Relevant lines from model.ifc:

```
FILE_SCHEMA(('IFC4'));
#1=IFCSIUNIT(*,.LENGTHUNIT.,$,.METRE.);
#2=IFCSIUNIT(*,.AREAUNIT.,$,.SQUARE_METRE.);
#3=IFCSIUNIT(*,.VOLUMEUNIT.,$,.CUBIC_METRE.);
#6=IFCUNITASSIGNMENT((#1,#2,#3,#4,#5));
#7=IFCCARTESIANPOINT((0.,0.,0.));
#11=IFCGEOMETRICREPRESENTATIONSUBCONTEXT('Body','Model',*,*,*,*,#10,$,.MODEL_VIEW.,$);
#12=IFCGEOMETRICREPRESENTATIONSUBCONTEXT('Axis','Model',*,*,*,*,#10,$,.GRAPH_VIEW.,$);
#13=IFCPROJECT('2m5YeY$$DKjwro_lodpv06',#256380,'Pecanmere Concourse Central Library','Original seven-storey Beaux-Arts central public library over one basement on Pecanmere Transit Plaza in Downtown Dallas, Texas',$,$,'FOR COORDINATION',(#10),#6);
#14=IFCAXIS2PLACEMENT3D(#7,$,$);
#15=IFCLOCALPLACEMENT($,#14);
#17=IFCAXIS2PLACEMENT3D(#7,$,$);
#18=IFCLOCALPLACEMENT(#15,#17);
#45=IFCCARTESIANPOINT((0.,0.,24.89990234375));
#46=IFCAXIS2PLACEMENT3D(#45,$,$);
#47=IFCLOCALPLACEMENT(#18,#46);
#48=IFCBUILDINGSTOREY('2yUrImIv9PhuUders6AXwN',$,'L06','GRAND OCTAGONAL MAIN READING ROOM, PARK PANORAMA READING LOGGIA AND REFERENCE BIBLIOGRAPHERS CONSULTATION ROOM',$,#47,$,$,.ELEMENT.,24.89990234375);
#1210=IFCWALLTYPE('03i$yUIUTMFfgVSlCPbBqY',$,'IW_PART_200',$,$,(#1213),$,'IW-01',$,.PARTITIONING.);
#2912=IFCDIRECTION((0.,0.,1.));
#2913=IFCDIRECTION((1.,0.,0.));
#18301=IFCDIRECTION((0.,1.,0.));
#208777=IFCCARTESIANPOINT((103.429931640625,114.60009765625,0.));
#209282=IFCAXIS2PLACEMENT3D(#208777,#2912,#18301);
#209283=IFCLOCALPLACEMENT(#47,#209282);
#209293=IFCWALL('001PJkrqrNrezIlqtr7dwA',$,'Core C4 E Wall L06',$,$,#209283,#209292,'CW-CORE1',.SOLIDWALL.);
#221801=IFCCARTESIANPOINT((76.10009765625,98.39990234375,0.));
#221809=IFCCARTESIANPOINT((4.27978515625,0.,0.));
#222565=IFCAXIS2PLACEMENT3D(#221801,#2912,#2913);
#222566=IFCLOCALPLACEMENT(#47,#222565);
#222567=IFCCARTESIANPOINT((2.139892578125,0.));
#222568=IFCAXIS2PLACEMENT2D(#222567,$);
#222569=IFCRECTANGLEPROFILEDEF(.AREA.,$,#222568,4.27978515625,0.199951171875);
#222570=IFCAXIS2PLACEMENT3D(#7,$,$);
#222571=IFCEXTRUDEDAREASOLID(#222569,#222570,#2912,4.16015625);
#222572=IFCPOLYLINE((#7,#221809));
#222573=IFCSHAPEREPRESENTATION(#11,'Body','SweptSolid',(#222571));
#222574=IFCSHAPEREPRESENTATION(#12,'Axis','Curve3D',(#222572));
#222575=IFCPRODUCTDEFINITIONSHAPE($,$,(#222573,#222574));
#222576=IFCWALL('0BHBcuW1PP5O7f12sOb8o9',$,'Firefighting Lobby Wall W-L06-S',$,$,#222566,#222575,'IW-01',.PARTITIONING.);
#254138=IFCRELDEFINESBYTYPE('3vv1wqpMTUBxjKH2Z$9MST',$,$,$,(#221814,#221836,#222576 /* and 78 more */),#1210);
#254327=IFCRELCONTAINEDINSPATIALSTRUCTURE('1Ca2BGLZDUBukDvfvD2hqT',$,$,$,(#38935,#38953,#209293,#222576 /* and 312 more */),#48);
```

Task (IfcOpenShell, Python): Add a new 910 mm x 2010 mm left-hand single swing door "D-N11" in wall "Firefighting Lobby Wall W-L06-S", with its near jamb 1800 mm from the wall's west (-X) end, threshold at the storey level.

```python
import numpy as np
import ifcopenshell
import ifcopenshell.api.feature
import ifcopenshell.api.geometry
import ifcopenshell.api.root
import ifcopenshell.api.spatial
import ifcopenshell.geom
import ifcopenshell.util.element
import ifcopenshell.util.placement
import ifcopenshell.util.representation
import ifcopenshell.util.shape
import ifcopenshell.util.unit

model = ifcopenshell.open("model.ifc")
unit_scale = ifcopenshell.util.unit.calculate_unit_scale(model)
settings = ifcopenshell.geom.settings()


def volume(element):
    """Net volume in cubic metres, openings subtracted."""
    shape = ifcopenshell.geom.create_shape(settings, element)
    return ifcopenshell.util.shape.get_volume(shape.geometry)


wall = model.by_guid("0BHBcuW1PP5O7f12sOb8o9")
storey = ifcopenshell.util.element.get_container(wall, ifc_class="IfcBuildingStorey")
context = ifcopenshell.util.representation.get_context(model, "Model", "Body", "MODEL_VIEW")
before = volume(wall)

width, height, from_end, sill = 0.91, 2.01, 1.8, 0.0  # metres

# The wall runs along its own X axis, and the end named is its -X end.
wall_shape = ifcopenshell.geom.create_shape(settings, wall)
x, y, z = ifcopenshell.util.shape.get_vertices(wall_shape.geometry).T
start = x.min() + from_end
face, thickness = float(y.min()), float(y.max() - y.min())
wall_matrix = ifcopenshell.util.placement.get_local_placement(wall.ObjectPlacement)
level = ifcopenshell.util.placement.get_local_placement(storey.ObjectPlacement)[2, 3]


def in_wall(x, y):
    """Placement at x, y metres in the wall's axes, at sill height."""
    matrix = wall_matrix.copy()
    matrix[:, 3] = wall_matrix @ np.array([x / unit_scale, y / unit_scale, 0.0, 1.0])
    matrix[2, 3] = level + sill / unit_scale
    return matrix


# Opening: a box that overshoots both wall faces by 50 mm.
opening = ifcopenshell.api.root.create_entity(model, ifc_class="IfcOpeningElement", predefined_type="OPENING")
box = ifcopenshell.api.geometry.add_wall_representation(
    model, context=context, length=width, height=height, thickness=thickness + 0.1
)
ifcopenshell.api.geometry.assign_representation(model, product=opening, representation=box)
ifcopenshell.api.geometry.edit_object_placement(model, product=opening, matrix=in_wall(start, face - 0.05), is_si=False)
ifcopenshell.api.feature.add_feature(model, feature=opening, element=wall)

door = ifcopenshell.api.root.create_entity(model, ifc_class="IfcDoor", name="D-N11", predefined_type="DOOR")
door.OverallWidth, door.OverallHeight = width / unit_scale, height / unit_scale
door.OperationType = "SINGLE_SWING_LEFT"
body = ifcopenshell.api.geometry.add_door_representation(
    model,
    context=context,
    overall_width=door.OverallWidth,
    overall_height=door.OverallHeight,
    operation_type="SINGLE_SWING_LEFT",
    lining_properties={"LiningDepth": thickness / unit_scale, "ThresholdDepth": thickness / unit_scale},
)
ifcopenshell.api.geometry.assign_representation(model, product=door, representation=body)
ifcopenshell.api.spatial.assign_container(model, products=[door], relating_structure=storey)
ifcopenshell.api.feature.add_filling(model, opening=opening, element=door)

# The lining spans the wall, so the door starts at the wall face.
ifcopenshell.api.geometry.edit_object_placement(model, product=door, matrix=in_wall(start, face), is_si=False)

after = volume(wall)

print(f"wall volume {before:.3f} -> {after:.3f} m3")

model.write("model_rev.ifc")
```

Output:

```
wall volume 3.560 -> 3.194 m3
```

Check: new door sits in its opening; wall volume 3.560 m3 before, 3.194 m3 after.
